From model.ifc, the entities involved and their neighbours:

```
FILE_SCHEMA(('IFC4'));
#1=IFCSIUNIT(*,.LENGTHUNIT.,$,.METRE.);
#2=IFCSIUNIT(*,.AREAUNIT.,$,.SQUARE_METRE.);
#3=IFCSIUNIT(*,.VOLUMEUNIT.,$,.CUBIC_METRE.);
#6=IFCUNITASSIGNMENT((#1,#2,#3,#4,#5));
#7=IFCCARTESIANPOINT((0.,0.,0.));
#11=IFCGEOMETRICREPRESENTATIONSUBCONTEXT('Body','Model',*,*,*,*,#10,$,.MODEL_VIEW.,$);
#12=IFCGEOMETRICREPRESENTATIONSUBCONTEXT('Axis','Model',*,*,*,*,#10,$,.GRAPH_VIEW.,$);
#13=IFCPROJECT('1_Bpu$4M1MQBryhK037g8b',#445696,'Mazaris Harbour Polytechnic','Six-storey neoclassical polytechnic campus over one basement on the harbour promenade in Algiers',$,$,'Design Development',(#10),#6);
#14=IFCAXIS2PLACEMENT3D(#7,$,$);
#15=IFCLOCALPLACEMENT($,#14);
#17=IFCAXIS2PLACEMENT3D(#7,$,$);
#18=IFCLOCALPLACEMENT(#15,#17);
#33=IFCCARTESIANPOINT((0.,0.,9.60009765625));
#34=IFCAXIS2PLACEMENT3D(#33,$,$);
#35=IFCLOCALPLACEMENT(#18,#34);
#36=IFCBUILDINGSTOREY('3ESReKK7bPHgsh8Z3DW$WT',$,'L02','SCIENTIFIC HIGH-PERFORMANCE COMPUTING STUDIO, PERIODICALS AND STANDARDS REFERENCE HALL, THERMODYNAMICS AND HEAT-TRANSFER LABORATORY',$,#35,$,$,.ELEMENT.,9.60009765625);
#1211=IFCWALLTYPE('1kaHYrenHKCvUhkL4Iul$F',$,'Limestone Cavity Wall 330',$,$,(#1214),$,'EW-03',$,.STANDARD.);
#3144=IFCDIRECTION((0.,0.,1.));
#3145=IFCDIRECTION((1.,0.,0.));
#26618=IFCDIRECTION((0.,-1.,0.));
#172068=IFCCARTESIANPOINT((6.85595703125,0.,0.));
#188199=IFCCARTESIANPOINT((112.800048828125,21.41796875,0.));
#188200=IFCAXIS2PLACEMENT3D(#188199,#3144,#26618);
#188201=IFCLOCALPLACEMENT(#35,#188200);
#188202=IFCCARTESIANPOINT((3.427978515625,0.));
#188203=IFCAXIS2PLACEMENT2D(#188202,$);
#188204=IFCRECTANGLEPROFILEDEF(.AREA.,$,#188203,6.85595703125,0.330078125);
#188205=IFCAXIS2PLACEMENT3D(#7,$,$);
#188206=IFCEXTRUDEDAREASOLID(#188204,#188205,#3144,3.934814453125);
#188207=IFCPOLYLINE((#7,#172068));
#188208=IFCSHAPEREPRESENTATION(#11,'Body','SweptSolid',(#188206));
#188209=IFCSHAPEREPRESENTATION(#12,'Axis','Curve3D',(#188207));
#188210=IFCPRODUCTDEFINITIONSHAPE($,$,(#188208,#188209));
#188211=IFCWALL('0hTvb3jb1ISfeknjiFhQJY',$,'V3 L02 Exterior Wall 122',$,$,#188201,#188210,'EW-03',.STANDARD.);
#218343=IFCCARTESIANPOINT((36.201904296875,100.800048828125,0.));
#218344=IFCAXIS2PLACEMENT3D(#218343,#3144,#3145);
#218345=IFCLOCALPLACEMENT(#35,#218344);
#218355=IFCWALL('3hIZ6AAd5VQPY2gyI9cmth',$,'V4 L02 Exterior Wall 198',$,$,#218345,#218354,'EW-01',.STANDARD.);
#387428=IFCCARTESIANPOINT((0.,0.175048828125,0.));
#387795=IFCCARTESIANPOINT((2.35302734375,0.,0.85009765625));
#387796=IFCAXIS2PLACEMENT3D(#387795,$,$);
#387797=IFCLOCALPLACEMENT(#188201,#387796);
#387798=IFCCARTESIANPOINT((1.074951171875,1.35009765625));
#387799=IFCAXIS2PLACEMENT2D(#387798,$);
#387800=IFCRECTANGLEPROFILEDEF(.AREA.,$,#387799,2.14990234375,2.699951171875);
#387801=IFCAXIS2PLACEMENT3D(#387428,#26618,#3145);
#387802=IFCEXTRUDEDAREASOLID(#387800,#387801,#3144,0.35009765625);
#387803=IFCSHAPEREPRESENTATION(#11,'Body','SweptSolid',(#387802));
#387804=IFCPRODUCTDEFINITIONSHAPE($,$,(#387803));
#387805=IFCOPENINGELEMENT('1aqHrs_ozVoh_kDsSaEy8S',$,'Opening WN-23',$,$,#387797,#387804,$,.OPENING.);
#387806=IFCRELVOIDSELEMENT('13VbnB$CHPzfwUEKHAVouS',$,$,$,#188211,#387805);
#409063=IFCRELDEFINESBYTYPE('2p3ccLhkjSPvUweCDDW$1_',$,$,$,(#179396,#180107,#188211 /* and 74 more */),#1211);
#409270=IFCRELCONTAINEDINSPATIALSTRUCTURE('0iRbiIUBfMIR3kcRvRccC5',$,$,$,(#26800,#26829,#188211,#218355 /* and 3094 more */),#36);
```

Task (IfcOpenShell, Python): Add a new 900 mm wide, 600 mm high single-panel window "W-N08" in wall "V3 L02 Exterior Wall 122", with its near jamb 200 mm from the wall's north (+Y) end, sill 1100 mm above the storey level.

```python
import numpy as np
import ifcopenshell
import ifcopenshell.api.feature
import ifcopenshell.api.geometry
import ifcopenshell.api.root
import ifcopenshell.api.spatial
import ifcopenshell.geom
import ifcopenshell.util.element
import ifcopenshell.util.placement
import ifcopenshell.util.representation
import ifcopenshell.util.shape
import ifcopenshell.util.unit

model = ifcopenshell.open("model.ifc")
unit_scale = ifcopenshell.util.unit.calculate_unit_scale(model)
settings = ifcopenshell.geom.settings()


def volume(element):
    """Net volume in cubic metres, openings subtracted."""
    shape = ifcopenshell.geom.create_shape(settings, element)
    return ifcopenshell.util.shape.get_volume(shape.geometry)


wall = model.by_guid("0hTvb3jb1ISfeknjiFhQJY")
storey = ifcopenshell.util.element.get_container(wall, ifc_class="IfcBuildingStorey")
context = ifcopenshell.util.representation.get_context(model, "Model", "Body", "MODEL_VIEW")
before = volume(wall)

width, height, from_end, sill = 0.9, 0.6, 0.2, 1.1  # metres

# The wall runs along its own X axis, and the end named is its -X end.
wall_shape = ifcopenshell.geom.create_shape(settings, wall)
x, y, z = ifcopenshell.util.shape.get_vertices(wall_shape.geometry).T
start = x.min() + from_end
face, thickness = float(y.min()), float(y.max() - y.min())
wall_matrix = ifcopenshell.util.placement.get_local_placement(wall.ObjectPlacement)
level = ifcopenshell.util.placement.get_local_placement(storey.ObjectPlacement)[2, 3]


def in_wall(x, y):
    """Placement at x, y metres in the wall's axes, at sill height."""
    matrix = wall_matrix.copy()
    matrix[:, 3] = wall_matrix @ np.array([x / unit_scale, y / unit_scale, 0.0, 1.0])
    matrix[2, 3] = level + sill / unit_scale
    return matrix


# Opening: a box that overshoots both wall faces by 50 mm.
opening = ifcopenshell.api.root.create_entity(model, ifc_class="IfcOpeningElement", predefined_type="OPENING")
box = ifcopenshell.api.geometry.add_wall_representation(
    model, context=context, length=width, height=height, thickness=thickness + 0.1
)
ifcopenshell.api.geometry.assign_representation(model, product=opening, representation=box)
ifcopenshell.api.geometry.edit_object_placement(model, product=opening, matrix=in_wall(start, face - 0.05), is_si=False)
ifcopenshell.api.feature.add_feature(model, feature=opening, element=wall)

window = ifcopenshell.api.root.create_entity(model, ifc_class="IfcWindow", name="W-N08", predefined_type="WINDOW")
window.OverallWidth, window.OverallHeight = width / unit_scale, height / unit_scale
window.PartitioningType = "SINGLE_PANEL"
body = ifcopenshell.api.geometry.add_window_representation(
    model,
    context=context,
    overall_width=window.OverallWidth,
    overall_height=window.OverallHeight,
    partition_type="SINGLE_PANEL",
)
ifcopenshell.api.geometry.assign_representation(model, product=window, representation=body)
ifcopenshell.api.spatial.assign_container(model, products=[window], relating_structure=storey)
ifcopenshell.api.feature.add_filling(model, opening=opening, element=window)

# Centre the window in the wall's thickness.
ifcopenshell.api.geometry.edit_object_placement(model, product=window, matrix=in_wall(start, face), is_si=False)
window_shape = ifcopenshell.geom.create_shape(settings, window)
depth = ifcopenshell.util.shape.get_vertices(window_shape.geometry)[:, 1]
offset = face + thickness / 2 - (depth.min() + depth.max()) / 2
ifcopenshell.api.geometry.edit_object_placement(model, product=window, matrix=in_wall(start, offset), is_si=False)

after = volume(wall)

print(f"wall volume {before:.3f} -> {after:.3f} m3")

model.write("model-out.ifc")
```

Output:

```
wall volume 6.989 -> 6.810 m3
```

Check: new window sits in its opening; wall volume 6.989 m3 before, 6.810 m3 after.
